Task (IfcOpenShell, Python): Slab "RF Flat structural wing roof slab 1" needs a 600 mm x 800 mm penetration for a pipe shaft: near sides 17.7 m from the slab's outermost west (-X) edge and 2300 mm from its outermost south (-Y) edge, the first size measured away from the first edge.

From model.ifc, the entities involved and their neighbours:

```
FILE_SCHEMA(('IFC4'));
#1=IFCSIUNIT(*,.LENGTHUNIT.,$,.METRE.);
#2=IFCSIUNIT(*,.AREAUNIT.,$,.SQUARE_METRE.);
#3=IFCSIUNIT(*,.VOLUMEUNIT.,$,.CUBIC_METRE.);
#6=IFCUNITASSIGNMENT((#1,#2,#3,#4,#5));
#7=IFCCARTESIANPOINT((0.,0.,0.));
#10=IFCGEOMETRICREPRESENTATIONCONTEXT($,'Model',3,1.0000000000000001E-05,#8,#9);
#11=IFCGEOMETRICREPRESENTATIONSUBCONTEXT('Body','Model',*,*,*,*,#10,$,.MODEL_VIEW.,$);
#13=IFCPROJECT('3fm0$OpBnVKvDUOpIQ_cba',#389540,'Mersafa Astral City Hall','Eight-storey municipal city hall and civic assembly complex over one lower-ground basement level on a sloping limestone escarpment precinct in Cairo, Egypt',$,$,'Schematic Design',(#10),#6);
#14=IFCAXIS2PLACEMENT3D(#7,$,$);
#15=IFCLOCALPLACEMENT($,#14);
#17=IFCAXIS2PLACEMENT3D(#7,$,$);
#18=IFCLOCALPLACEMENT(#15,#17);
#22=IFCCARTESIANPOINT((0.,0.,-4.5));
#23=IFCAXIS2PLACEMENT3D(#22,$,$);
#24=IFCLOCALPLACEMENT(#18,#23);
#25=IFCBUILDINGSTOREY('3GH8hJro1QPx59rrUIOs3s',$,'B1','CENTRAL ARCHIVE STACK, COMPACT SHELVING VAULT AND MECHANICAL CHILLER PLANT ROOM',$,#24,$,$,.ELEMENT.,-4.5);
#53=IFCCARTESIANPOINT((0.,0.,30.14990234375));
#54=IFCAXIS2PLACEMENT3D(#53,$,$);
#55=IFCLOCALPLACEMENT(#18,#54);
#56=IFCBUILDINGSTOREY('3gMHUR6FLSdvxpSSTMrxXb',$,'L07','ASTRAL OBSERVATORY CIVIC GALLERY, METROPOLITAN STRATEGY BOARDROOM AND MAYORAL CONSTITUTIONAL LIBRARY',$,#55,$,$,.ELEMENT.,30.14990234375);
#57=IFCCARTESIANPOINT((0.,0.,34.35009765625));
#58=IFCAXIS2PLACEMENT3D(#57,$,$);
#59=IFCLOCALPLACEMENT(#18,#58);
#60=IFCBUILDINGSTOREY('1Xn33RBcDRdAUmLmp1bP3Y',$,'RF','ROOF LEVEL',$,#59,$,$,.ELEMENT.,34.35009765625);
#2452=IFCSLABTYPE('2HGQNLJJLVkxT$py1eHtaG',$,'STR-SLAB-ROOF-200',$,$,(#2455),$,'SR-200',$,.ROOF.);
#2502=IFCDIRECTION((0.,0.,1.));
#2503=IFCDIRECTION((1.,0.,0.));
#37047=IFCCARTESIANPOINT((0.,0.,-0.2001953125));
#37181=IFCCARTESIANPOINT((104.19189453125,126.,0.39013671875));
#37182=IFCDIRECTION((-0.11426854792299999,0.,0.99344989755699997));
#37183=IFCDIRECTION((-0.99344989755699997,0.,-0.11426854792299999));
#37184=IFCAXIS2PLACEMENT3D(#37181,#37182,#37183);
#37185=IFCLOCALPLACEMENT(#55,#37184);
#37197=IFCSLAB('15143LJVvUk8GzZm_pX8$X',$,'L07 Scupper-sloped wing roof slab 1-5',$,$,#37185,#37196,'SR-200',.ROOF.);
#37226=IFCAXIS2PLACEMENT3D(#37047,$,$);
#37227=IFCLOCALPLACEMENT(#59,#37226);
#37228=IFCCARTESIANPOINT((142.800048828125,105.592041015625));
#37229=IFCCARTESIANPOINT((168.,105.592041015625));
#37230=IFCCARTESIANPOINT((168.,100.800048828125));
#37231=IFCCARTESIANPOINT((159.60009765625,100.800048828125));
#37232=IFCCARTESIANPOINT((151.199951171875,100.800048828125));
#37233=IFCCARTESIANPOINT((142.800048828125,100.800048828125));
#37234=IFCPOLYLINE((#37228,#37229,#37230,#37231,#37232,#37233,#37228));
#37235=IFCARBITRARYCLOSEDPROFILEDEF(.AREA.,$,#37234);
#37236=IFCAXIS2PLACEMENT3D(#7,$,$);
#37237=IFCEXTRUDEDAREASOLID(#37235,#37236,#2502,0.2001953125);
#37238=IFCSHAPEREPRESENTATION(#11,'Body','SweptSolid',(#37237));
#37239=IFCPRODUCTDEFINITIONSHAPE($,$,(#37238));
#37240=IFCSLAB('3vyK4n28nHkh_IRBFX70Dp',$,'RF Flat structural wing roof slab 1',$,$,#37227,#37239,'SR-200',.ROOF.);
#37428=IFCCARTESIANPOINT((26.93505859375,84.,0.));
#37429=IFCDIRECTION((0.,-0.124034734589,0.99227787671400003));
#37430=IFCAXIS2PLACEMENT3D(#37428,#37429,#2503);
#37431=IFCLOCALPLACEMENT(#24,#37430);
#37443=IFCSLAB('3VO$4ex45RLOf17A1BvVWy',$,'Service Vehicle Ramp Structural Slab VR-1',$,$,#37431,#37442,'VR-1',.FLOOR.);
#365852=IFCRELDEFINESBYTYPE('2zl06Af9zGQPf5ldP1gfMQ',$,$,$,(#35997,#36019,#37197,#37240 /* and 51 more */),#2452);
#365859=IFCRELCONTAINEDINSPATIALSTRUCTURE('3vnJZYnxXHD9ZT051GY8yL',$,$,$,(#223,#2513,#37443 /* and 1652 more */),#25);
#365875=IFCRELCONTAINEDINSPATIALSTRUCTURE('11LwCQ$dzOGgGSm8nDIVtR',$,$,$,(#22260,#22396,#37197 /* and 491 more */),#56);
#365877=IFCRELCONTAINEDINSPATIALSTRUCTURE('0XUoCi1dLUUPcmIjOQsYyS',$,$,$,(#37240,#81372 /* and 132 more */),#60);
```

```python
import numpy as np
import ifcopenshell
import ifcopenshell.api.feature
import ifcopenshell.api.geometry
import ifcopenshell.api.root
import ifcopenshell.geom
import ifcopenshell.util.placement
import ifcopenshell.util.representation
import ifcopenshell.util.shape
import ifcopenshell.util.unit

model = ifcopenshell.open("model.ifc")
unit_scale = ifcopenshell.util.unit.calculate_unit_scale(model)
settings = ifcopenshell.geom.settings()


def volume(element):
    """Net volume in cubic metres, openings subtracted."""
    shape = ifcopenshell.geom.create_shape(settings, element)
    return ifcopenshell.util.shape.get_volume(shape.geometry)


slab = model.by_guid("3vyK4n28nHkh_IRBFX70Dp")
before = volume(slab)

# Extent in the slab's own axes, in metres. The edges named are its -X and -Y sides.
slab_shape = ifcopenshell.geom.create_shape(settings, slab)
vertices = ifcopenshell.util.shape.get_vertices(slab_shape.geometry)
x_min, y_min, bottom = vertices.min(axis=0)
top = vertices[:, 2].max()

opening = ifcopenshell.api.root.create_entity(model, ifc_class="IfcOpeningElement", name="Pipe shaft opening", predefined_type="OPENING")
context = ifcopenshell.util.representation.get_context(model, "Model", "Body", "MODEL_VIEW")
width, depth = 0.6, 0.8
outline = [(0.0, 0.0), (width, 0.0), (width, depth), (0.0, depth), (0.0, 0.0)]
# Overshoot both faces by 50 mm so the cut is clean.
shape = ifcopenshell.api.geometry.add_slab_representation(
    model, context=context, depth=top - bottom + 0.1, polyline=outline
)
ifcopenshell.api.geometry.assign_representation(model, product=opening, representation=shape)

matrix = ifcopenshell.util.placement.get_local_placement(slab.ObjectPlacement)
matrix[:, 3] = matrix @ np.append(np.array([x_min + 17.7, y_min + 2.3, bottom - 0.05]) / unit_scale, 1.0)
ifcopenshell.api.geometry.edit_object_placement(model, product=opening, matrix=matrix, is_si=False)
ifcopenshell.api.feature.add_feature(model, feature=opening, element=slab)

after = volume(slab)

print(f"slab volume {before:.3f} -> {after:.3f} m3")

model.write("model_v2.ifc")
```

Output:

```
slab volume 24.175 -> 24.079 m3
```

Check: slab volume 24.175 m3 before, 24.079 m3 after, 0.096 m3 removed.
